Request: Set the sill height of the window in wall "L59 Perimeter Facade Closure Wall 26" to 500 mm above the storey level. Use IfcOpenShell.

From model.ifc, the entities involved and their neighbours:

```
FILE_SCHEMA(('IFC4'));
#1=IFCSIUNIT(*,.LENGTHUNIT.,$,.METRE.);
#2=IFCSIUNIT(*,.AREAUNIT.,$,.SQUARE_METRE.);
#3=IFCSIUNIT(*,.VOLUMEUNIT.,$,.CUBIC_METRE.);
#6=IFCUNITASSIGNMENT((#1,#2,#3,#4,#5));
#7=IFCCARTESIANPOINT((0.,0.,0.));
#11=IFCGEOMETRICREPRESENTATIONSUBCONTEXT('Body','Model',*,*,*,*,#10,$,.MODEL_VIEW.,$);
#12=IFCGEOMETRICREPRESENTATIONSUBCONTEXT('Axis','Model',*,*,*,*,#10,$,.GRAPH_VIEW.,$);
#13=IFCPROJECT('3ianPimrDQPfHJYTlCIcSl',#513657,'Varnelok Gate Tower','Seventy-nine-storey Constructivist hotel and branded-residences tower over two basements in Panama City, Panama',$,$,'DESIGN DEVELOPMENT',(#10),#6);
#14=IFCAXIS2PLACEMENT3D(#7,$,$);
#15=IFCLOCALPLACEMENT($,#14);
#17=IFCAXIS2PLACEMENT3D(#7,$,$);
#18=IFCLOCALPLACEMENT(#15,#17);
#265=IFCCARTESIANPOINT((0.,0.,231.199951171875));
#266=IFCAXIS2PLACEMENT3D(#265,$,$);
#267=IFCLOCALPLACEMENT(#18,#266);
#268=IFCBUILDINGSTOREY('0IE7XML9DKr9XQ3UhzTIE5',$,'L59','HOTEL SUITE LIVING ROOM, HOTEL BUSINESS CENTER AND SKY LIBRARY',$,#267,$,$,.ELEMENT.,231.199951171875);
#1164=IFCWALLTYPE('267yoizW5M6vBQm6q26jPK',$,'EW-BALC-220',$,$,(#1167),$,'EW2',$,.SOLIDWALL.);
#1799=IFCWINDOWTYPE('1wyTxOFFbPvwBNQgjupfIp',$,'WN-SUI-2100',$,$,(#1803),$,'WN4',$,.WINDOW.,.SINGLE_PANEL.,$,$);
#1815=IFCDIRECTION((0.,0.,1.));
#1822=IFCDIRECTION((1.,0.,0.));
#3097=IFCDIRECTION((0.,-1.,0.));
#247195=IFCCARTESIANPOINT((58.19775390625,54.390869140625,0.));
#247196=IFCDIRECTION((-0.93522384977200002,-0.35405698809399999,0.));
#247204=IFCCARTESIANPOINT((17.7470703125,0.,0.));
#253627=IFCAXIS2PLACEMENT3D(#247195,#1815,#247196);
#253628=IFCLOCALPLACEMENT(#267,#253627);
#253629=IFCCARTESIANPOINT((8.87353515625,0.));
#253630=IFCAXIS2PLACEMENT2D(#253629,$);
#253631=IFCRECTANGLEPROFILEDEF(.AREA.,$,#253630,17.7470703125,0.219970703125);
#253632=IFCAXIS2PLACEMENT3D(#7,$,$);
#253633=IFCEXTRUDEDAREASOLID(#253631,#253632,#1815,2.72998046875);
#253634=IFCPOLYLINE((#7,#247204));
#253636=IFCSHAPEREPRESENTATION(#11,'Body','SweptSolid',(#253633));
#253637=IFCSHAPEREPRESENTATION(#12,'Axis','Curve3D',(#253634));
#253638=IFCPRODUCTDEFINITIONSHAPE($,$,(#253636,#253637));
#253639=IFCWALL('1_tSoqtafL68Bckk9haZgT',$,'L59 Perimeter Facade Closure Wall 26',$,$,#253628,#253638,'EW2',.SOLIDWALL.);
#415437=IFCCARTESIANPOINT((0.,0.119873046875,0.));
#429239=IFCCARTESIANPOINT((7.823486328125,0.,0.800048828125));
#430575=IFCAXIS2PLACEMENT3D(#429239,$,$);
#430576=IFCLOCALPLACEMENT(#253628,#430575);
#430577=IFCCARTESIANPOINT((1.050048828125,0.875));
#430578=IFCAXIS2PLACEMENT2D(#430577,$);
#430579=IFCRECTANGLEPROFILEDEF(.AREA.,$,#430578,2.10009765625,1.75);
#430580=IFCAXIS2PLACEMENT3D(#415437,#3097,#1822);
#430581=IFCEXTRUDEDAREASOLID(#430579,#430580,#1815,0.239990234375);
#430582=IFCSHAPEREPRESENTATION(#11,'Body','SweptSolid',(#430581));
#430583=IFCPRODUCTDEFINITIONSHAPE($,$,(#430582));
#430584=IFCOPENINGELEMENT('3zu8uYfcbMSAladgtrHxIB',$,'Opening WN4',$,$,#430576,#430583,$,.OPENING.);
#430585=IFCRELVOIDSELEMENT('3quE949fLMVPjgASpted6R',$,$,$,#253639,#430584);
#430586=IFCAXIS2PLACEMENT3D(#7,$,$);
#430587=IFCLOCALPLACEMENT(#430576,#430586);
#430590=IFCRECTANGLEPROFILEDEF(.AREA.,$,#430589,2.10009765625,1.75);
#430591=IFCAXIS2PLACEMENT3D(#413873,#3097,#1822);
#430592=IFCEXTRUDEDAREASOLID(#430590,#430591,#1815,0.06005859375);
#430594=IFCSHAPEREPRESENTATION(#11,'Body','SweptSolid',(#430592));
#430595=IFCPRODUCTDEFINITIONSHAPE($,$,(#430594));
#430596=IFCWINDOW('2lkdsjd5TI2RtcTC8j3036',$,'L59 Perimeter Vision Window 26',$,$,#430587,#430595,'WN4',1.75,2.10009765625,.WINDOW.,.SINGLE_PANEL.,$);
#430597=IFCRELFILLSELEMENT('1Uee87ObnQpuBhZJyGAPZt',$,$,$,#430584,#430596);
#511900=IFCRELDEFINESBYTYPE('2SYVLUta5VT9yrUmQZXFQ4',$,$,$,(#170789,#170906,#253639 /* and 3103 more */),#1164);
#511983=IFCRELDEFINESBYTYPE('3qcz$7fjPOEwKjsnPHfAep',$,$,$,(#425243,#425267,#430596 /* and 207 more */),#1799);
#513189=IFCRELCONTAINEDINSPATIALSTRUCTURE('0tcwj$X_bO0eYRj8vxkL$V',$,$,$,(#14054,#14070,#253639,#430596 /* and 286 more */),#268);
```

```python
import numpy as np
import ifcopenshell
import ifcopenshell.api.geometry
import ifcopenshell.geom
import ifcopenshell.util.element
import ifcopenshell.util.placement
import ifcopenshell.util.shape
import ifcopenshell.util.unit

model = ifcopenshell.open("model.ifc")
unit_scale = ifcopenshell.util.unit.calculate_unit_scale(model)

window = model.by_guid("2lkdsjd5TI2RtcTC8j3036")
opening = window.FillsVoids[0].RelatingOpeningElement
storey = ifcopenshell.util.element.get_container(window, ifc_class="IfcBuildingStorey")
level = ifcopenshell.util.placement.get_local_placement(storey.ObjectPlacement)[2, 3]

# The opening's origin need not be at the sill, so measure its lowest point.
shape = ifcopenshell.geom.create_shape(ifcopenshell.geom.settings(), opening)
bottom = ifcopenshell.util.shape.get_shape_bottom_elevation(shape, shape.geometry) / unit_scale
dz = level + 0.5 / unit_scale - bottom

shift = np.array([0.0, 0.0, dz])
# The window is placed relative to its opening, so it follows when the opening moves.
matrix = ifcopenshell.util.placement.get_local_placement(opening.ObjectPlacement)
matrix[:3, 3] += shift
ifcopenshell.api.geometry.edit_object_placement(
    model, product=opening, matrix=matrix, is_si=False, should_transform_children=True
)

print(f"moved by {dz * unit_scale:+.3f} m")

model.write("model_v2.ifc")
```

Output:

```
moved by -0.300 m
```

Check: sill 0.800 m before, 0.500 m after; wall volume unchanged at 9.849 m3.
